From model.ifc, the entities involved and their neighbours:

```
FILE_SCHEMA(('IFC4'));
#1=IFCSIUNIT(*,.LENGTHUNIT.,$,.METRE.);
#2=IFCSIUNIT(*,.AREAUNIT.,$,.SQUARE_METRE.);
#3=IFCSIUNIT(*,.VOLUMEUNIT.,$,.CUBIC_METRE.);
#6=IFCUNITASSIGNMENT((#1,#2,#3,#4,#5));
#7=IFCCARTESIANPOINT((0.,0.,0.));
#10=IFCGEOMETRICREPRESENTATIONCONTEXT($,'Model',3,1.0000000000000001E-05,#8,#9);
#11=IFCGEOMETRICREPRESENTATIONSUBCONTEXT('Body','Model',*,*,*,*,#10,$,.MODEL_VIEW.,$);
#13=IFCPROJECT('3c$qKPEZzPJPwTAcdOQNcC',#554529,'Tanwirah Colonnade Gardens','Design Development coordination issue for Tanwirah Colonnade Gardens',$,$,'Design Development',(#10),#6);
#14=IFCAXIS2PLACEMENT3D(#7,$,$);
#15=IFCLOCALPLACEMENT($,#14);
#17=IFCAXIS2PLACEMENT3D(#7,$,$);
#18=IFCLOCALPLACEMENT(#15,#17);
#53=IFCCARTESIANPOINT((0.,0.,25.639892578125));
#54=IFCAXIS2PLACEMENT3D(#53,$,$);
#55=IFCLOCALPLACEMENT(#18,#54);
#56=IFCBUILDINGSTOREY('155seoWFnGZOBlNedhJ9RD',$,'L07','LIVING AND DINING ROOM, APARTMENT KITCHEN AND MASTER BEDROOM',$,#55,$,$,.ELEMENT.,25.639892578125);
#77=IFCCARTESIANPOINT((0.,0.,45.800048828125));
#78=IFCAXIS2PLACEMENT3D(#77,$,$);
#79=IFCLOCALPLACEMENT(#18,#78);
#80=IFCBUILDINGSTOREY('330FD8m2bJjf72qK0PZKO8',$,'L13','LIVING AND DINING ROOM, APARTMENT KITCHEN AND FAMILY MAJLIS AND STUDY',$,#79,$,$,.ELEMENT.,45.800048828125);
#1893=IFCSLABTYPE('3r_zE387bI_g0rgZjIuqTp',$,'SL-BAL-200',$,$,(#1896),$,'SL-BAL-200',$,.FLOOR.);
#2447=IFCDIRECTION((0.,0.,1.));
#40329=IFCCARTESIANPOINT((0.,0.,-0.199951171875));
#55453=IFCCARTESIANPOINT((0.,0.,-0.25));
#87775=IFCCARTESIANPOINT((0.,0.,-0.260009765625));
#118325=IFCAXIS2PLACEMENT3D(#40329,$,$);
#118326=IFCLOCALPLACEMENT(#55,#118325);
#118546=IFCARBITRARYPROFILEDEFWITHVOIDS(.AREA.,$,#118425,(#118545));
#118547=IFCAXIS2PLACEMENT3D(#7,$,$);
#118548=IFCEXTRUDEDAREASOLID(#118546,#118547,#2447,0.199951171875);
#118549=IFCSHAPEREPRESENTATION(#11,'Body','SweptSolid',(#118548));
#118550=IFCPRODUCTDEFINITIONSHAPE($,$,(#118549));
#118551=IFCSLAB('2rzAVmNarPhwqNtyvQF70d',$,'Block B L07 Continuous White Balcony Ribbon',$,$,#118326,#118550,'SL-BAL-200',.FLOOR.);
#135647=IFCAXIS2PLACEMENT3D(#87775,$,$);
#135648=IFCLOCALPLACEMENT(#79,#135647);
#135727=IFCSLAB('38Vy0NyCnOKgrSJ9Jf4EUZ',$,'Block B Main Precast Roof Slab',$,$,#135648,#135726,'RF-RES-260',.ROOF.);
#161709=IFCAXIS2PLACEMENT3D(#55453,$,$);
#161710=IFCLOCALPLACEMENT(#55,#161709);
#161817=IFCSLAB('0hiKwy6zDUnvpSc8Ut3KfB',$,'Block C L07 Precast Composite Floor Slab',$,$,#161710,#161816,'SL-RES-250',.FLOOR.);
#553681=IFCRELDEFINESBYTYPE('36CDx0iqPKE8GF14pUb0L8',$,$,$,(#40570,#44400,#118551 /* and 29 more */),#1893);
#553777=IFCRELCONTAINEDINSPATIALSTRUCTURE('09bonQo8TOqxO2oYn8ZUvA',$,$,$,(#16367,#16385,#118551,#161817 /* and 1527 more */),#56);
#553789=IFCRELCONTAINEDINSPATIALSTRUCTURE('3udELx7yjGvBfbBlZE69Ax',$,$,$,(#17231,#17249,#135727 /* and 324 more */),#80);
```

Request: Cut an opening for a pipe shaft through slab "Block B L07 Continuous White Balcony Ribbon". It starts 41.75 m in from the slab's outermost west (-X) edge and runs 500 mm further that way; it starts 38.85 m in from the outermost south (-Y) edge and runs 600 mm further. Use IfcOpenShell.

```python
import numpy as np
import ifcopenshell
import ifcopenshell.api.feature
import ifcopenshell.api.geometry
import ifcopenshell.api.root
import ifcopenshell.geom
import ifcopenshell.util.placement
import ifcopenshell.util.representation
import ifcopenshell.util.shape
import ifcopenshell.util.unit

model = ifcopenshell.open("model.ifc")
unit_scale = ifcopenshell.util.unit.calculate_unit_scale(model)
settings = ifcopenshell.geom.settings()


def volume(element):
    """Net volume in cubic metres, openings subtracted."""
    shape = ifcopenshell.geom.create_shape(settings, element)
    return ifcopenshell.util.shape.get_volume(shape.geometry)


slab = model.by_guid("2rzAVmNarPhwqNtyvQF70d")
before = volume(slab)

# Extent in the slab's own axes, in metres. The edges named are its -X and -Y sides.
slab_shape = ifcopenshell.geom.create_shape(settings, slab)
vertices = ifcopenshell.util.shape.get_vertices(slab_shape.geometry)
x_min, y_min, bottom = vertices.min(axis=0)
top = vertices[:, 2].max()

opening = ifcopenshell.api.root.create_entity(model, ifc_class="IfcOpeningElement", name="Pipe shaft opening", predefined_type="OPENING")
context = ifcopenshell.util.representation.get_context(model, "Model", "Body", "MODEL_VIEW")
width, depth = 0.5, 0.6
outline = [(0.0, 0.0), (width, 0.0), (width, depth), (0.0, depth), (0.0, 0.0)]
# Overshoot both faces by 50 mm so the cut is clean.
shape = ifcopenshell.api.geometry.add_slab_representation(
    model, context=context, depth=top - bottom + 0.1, polyline=outline
)
ifcopenshell.api.geometry.assign_representation(model, product=opening, representation=shape)

matrix = ifcopenshell.util.placement.get_local_placement(slab.ObjectPlacement)
matrix[:, 3] = matrix @ np.append(np.array([x_min + 41.75, y_min + 38.85, bottom - 0.05]) / unit_scale, 1.0)
ifcopenshell.api.geometry.edit_object_placement(model, product=opening, matrix=matrix, is_si=False)
ifcopenshell.api.feature.add_feature(model, feature=opening, element=slab)

after = volume(slab)

print(f"slab volume {before:.3f} -> {after:.3f} m3")

model.write("model_rev.ifc")
```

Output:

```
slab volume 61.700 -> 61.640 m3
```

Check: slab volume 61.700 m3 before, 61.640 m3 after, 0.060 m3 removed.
